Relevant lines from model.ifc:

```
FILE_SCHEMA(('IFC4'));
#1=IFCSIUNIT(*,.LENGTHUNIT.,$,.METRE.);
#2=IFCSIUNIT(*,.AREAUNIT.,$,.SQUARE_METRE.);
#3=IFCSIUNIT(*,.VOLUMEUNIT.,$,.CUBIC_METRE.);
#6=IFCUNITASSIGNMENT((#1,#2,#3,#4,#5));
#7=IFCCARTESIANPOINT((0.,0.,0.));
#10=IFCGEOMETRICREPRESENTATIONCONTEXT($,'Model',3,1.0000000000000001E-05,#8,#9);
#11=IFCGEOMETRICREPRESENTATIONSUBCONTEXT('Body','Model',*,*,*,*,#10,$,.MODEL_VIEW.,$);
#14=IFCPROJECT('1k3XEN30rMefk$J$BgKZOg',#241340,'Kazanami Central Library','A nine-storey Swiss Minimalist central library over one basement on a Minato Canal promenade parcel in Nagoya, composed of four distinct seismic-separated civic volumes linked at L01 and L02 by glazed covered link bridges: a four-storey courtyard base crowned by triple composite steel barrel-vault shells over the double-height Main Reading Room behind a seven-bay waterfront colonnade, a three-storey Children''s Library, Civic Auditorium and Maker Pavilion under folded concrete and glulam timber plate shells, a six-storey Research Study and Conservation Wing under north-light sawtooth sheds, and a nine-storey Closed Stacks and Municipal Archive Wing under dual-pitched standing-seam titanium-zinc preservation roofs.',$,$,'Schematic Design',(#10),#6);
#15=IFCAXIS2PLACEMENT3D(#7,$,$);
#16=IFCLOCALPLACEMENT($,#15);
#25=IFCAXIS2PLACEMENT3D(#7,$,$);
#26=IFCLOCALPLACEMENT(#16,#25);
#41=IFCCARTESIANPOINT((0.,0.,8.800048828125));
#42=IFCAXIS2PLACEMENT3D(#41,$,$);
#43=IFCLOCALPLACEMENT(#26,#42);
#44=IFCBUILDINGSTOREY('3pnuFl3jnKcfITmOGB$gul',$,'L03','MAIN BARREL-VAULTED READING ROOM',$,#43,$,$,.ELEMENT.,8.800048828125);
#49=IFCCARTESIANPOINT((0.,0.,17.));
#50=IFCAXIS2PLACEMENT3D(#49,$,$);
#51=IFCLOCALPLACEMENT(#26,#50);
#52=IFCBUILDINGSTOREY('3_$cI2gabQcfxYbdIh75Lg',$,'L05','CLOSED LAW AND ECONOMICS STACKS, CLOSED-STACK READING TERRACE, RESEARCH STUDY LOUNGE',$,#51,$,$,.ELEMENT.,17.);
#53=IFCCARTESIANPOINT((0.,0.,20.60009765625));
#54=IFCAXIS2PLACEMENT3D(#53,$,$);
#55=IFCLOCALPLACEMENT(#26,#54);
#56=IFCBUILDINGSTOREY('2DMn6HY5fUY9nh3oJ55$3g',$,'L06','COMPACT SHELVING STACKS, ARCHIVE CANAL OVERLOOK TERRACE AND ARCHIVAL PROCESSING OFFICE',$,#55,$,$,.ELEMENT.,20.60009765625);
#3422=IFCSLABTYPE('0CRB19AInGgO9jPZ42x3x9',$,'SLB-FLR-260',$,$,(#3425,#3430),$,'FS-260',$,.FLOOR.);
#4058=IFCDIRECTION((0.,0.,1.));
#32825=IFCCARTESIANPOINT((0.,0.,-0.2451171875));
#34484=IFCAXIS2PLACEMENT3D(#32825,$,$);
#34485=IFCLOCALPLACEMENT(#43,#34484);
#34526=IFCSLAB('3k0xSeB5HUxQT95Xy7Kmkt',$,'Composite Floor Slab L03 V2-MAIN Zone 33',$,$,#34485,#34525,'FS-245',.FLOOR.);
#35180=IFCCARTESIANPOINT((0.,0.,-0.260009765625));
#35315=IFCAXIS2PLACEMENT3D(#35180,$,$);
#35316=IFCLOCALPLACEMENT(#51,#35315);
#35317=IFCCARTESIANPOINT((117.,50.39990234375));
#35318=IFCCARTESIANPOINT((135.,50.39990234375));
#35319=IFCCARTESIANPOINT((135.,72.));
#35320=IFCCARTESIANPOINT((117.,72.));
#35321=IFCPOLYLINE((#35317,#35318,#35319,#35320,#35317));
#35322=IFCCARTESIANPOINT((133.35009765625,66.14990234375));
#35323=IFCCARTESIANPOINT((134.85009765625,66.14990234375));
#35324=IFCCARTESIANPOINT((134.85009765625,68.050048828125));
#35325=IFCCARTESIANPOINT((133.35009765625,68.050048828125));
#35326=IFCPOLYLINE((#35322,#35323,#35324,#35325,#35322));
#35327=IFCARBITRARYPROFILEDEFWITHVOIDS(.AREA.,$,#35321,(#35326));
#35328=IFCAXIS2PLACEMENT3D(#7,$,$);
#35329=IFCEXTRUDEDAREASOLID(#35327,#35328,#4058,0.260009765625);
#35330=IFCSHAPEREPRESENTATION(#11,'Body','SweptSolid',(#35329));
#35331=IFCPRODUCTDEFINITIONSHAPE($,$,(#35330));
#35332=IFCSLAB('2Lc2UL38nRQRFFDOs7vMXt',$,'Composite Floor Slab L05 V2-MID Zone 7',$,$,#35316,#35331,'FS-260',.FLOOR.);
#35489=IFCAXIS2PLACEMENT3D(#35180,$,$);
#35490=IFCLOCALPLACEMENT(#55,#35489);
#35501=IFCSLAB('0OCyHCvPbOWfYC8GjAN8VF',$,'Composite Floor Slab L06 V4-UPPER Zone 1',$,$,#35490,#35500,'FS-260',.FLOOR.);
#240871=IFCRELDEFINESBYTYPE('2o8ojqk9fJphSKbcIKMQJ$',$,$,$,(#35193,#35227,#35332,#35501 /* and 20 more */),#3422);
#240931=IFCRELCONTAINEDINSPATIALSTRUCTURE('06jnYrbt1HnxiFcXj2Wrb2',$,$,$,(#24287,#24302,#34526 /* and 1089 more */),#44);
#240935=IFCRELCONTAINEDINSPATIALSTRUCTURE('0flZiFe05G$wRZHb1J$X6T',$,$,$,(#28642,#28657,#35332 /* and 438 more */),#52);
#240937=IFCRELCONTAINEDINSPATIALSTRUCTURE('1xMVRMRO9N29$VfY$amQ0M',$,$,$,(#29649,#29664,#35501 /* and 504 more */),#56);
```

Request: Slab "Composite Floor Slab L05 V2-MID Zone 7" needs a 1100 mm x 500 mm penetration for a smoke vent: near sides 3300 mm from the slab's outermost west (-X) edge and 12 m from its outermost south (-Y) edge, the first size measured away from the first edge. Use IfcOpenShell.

```python
import numpy as np
import ifcopenshell
import ifcopenshell.api.feature
import ifcopenshell.api.geometry
import ifcopenshell.api.root
import ifcopenshell.geom
import ifcopenshell.util.placement
import ifcopenshell.util.representation
import ifcopenshell.util.shape
import ifcopenshell.util.unit

model = ifcopenshell.open("model.ifc")
unit_scale = ifcopenshell.util.unit.calculate_unit_scale(model)
settings = ifcopenshell.geom.settings()


def volume(element):
    """Net volume in cubic metres, openings subtracted."""
    shape = ifcopenshell.geom.create_shape(settings, element)
    return ifcopenshell.util.shape.get_volume(shape.geometry)


slab = model.by_id(35332)
before = volume(slab)

# Extent in the slab's own axes, in metres. The edges named are its -X and -Y sides.
slab_shape = ifcopenshell.geom.create_shape(settings, slab)
vertices = ifcopenshell.util.shape.get_vertices(slab_shape.geometry)
x_min, y_min, bottom = vertices.min(axis=0)
top = vertices[:, 2].max()

opening = ifcopenshell.api.root.create_entity(model, ifc_class="IfcOpeningElement", name="Smoke vent opening", predefined_type="OPENING")
context = ifcopenshell.util.representation.get_context(model, "Model", "Body", "MODEL_VIEW")
width, depth = 1.1, 0.5
outline = [(0.0, 0.0), (width, 0.0), (width, depth), (0.0, depth), (0.0, 0.0)]
# Overshoot both faces by 50 mm so the cut is clean.
shape = ifcopenshell.api.geometry.add_slab_representation(
    model, context=context, depth=top - bottom + 0.1, polyline=outline
)
ifcopenshell.api.geometry.assign_representation(model, product=opening, representation=shape)

matrix = ifcopenshell.util.placement.get_local_placement(slab.ObjectPlacement)
matrix[:, 3] = matrix @ np.append(np.array([x_min + 3.3, y_min + 12, bottom - 0.05]) / unit_scale, 1.0)
ifcopenshell.api.geometry.edit_object_placement(model, product=opening, matrix=matrix, is_si=False)
ifcopenshell.api.feature.add_feature(model, feature=opening, element=slab)

after = volume(slab)

print(f"slab volume {before:.3f} -> {after:.3f} m3")

model.write("model_v2.ifc")
```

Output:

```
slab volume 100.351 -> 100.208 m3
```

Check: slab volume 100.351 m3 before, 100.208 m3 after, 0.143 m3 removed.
